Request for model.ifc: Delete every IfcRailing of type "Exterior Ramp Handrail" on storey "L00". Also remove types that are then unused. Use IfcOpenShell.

First a look at what the model holds.

```python
import ifcopenshell
import ifcopenshell.util.element

model = ifcopenshell.open("model.ifc")
print(model.schema)
storey = next(s for s in model.by_type("IfcBuildingStorey") if s.Name == "L00")
railings = [e for e in ifcopenshell.util.element.get_decomposition(storey) if e.is_a("IfcRailing")]
seen = {}
for e in railings:
    element_type = ifcopenshell.util.element.get_type(e)
    name = element_type.Name if element_type not in (None, e) else None
    seen[name] = seen.get(name, 0) + 1
for name, count in sorted(seen.items(), key=str):
    print(count, "x", name)
```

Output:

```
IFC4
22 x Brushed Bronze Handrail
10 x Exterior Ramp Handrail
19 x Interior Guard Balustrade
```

```python
import ifcopenshell
import ifcopenshell.api.root
import ifcopenshell.util.element

model = ifcopenshell.open("model.ifc")

storey = next(s for s in model.by_type("IfcBuildingStorey") if s.Name == "L00")
railings = [e for e in ifcopenshell.util.element.get_decomposition(storey) if e.is_a("IfcRailing")]
targets = [e for e in railings if (t := ifcopenshell.util.element.get_type(e)) not in (None, e) and t.Name == "Exterior Ramp Handrail"]
types = {ifcopenshell.util.element.get_type(e) for e in targets} - {None, *targets}

for e in targets:
    ifcopenshell.api.root.remove_product(model, product=e)
print(len(targets), "removed")

unused = [t for t in types if not ifcopenshell.util.element.get_types(t)]
for t in unused:
    ifcopenshell.api.root.remove_product(model, product=t)
print(len(unused), "unused types removed")

model.write("model_rev.ifc")
```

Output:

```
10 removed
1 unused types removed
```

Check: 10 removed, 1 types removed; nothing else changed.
